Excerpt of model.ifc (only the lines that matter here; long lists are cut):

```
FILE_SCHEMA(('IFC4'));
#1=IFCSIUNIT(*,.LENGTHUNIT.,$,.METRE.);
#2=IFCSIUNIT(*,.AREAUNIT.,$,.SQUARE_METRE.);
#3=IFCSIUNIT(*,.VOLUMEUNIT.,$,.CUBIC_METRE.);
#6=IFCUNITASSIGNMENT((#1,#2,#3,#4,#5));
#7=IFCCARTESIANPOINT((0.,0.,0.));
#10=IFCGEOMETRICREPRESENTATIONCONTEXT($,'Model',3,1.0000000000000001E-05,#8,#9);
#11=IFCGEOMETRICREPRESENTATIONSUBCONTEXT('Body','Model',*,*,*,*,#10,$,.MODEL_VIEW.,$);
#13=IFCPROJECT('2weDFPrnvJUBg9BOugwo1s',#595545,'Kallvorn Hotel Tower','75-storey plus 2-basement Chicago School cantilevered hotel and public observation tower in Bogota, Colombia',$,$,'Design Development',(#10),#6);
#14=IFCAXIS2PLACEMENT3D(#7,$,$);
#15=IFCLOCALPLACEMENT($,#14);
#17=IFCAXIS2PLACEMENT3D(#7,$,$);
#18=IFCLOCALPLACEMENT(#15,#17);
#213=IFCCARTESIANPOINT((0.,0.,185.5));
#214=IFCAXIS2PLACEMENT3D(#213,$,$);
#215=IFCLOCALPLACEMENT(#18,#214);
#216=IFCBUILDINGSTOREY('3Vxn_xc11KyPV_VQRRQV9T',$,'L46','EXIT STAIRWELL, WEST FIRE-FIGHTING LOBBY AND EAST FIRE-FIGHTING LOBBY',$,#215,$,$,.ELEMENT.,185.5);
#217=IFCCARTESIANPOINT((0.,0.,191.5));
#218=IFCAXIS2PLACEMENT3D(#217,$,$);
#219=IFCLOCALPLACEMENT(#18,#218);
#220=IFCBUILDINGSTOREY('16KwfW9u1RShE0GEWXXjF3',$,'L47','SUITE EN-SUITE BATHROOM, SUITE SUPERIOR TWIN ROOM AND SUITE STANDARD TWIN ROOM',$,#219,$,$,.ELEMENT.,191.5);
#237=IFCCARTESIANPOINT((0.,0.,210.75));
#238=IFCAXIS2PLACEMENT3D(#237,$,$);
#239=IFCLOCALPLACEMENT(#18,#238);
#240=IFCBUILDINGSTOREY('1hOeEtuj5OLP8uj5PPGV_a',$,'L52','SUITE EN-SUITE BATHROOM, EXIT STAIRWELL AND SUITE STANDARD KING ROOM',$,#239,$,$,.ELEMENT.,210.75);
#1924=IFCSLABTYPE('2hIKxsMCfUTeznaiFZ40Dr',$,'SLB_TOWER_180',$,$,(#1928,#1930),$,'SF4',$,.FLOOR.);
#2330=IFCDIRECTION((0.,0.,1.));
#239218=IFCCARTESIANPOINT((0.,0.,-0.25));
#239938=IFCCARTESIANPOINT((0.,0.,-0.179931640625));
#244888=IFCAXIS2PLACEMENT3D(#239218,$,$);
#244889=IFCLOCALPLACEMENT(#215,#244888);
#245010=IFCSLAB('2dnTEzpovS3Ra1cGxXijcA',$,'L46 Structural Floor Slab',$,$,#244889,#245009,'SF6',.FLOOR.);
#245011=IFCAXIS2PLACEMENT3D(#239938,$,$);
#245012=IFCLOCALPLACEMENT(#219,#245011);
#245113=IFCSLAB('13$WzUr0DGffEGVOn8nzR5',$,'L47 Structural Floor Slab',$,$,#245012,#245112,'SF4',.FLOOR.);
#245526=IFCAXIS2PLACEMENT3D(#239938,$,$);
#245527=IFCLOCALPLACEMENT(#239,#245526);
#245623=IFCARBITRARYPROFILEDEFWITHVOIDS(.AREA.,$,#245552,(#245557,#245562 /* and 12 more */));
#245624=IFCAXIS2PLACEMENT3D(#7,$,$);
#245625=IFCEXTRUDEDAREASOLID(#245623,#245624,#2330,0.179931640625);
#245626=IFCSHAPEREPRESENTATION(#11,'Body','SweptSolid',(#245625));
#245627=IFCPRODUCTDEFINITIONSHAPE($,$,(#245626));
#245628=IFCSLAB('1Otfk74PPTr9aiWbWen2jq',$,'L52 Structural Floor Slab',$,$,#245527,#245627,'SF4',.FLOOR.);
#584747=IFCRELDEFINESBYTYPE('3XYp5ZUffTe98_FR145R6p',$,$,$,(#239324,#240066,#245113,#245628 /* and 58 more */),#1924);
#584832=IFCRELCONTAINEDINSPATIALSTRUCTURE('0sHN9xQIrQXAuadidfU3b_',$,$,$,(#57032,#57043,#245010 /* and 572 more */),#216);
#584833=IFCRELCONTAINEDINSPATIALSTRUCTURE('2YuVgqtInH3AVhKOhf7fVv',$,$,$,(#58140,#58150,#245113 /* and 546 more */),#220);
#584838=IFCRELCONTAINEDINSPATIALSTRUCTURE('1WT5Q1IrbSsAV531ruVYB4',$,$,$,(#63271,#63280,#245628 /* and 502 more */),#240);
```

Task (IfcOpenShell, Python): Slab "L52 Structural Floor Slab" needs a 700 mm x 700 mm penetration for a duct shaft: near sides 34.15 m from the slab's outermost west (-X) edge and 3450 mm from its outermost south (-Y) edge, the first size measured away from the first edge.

```python
import numpy as np
import ifcopenshell
import ifcopenshell.api.feature
import ifcopenshell.api.geometry
import ifcopenshell.api.root
import ifcopenshell.geom
import ifcopenshell.util.placement
import ifcopenshell.util.representation
import ifcopenshell.util.shape
import ifcopenshell.util.unit

model = ifcopenshell.open("model.ifc")
unit_scale = ifcopenshell.util.unit.calculate_unit_scale(model)
settings = ifcopenshell.geom.settings()


def volume(element):
    """Net volume in cubic metres, openings subtracted."""
    shape = ifcopenshell.geom.create_shape(settings, element)
    return ifcopenshell.util.shape.get_volume(shape.geometry)


slab = model.by_guid("1Otfk74PPTr9aiWbWen2jq")
before = volume(slab)

# Extent in the slab's own axes, in metres. The edges named are its -X and -Y sides.
slab_shape = ifcopenshell.geom.create_shape(settings, slab)
vertices = ifcopenshell.util.shape.get_vertices(slab_shape.geometry)
x_min, y_min, bottom = vertices.min(axis=0)
top = vertices[:, 2].max()

opening = ifcopenshell.api.root.create_entity(model, ifc_class="IfcOpeningElement", name="Duct shaft opening", predefined_type="OPENING")
context = ifcopenshell.util.representation.get_context(model, "Model", "Body", "MODEL_VIEW")
width, depth = 0.7, 0.7
outline = [(0.0, 0.0), (width, 0.0), (width, depth), (0.0, depth), (0.0, 0.0)]
# Overshoot both faces by 50 mm so the cut is clean.
shape = ifcopenshell.api.geometry.add_slab_representation(
    model, context=context, depth=top - bottom + 0.1, polyline=outline
)
ifcopenshell.api.geometry.assign_representation(model, product=opening, representation=shape)

matrix = ifcopenshell.util.placement.get_local_placement(slab.ObjectPlacement)
matrix[:, 3] = matrix @ np.append(np.array([x_min + 34.15, y_min + 3.45, bottom - 0.05]) / unit_scale, 1.0)
ifcopenshell.api.geometry.edit_object_placement(model, product=opening, matrix=matrix, is_si=False)
ifcopenshell.api.feature.add_feature(model, feature=opening, element=slab)

after = volume(slab)

print(f"slab volume {before:.3f} -> {after:.3f} m3")

model.write("model-out.ifc")
```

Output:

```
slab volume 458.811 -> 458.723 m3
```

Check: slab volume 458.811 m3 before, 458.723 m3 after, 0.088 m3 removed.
